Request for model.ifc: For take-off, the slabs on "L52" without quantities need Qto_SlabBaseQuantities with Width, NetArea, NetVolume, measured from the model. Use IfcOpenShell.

First a look at what the model holds.

```python
import ifcopenshell
import ifcopenshell.util.element
import ifcopenshell.util.unit

model = ifcopenshell.open("model.ifc")
print(model.schema)
for unit_type in ("LENGTHUNIT", "AREAUNIT", "VOLUMEUNIT"):
    print(unit_type, ifcopenshell.util.unit.calculate_unit_scale(model, unit_type))
storey = next(s for s in model.by_type("IfcBuildingStorey") if s.Name == "L52")
slabs = [e for e in ifcopenshell.util.element.get_decomposition(storey) if e.is_a("IfcSlab")]
for e in sorted(slabs, key=lambda e: e.id()):
    print(e.id(), e.is_a(), e.Name, list(ifcopenshell.util.element.get_psets(e, qtos_only=True)), sep=" | ")
```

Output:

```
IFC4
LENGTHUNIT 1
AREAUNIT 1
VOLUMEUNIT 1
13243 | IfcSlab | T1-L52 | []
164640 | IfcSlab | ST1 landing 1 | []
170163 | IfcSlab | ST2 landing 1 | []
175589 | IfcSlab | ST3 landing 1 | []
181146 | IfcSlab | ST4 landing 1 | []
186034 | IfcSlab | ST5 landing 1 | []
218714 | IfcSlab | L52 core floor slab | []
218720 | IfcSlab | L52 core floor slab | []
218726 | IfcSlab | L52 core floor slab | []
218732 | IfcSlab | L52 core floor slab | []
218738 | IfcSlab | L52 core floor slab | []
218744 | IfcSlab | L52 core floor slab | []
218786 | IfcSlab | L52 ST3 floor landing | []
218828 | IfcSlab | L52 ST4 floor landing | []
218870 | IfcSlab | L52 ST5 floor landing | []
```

```python
import ifcopenshell
import ifcopenshell.api.pset
import ifcopenshell.geom
import ifcopenshell.util.element
import ifcopenshell.util.shape
import ifcopenshell.util.unit

model = ifcopenshell.open("model.ifc")
unit_scale = ifcopenshell.util.unit.calculate_unit_scale(model)
area_scale = ifcopenshell.util.unit.calculate_unit_scale(model, "AREAUNIT")
volume_scale = ifcopenshell.util.unit.calculate_unit_scale(model, "VOLUMEUNIT")
settings = ifcopenshell.geom.settings()

storey = next(s for s in model.by_type("IfcBuildingStorey") if s.Name == "L52")
slabs = [e for e in ifcopenshell.util.element.get_decomposition(storey) if e.is_a("IfcSlab")]

for e in sorted(slabs, key=lambda e: e.id()):
    if ifcopenshell.util.element.get_psets(e, qtos_only=True, should_inherit=False):
        continue
    # Geometry comes back in metres, in the element's own axes.
    shape = ifcopenshell.geom.create_shape(settings, e)
    values = {
        "Width": ifcopenshell.util.shape.get_z(shape.geometry) / unit_scale,
        "NetArea": ifcopenshell.util.shape.get_footprint_area(shape.geometry) / area_scale,
        "NetVolume": ifcopenshell.util.shape.get_volume(shape.geometry) / volume_scale,
    }
    qto = ifcopenshell.api.pset.add_qto(model, product=e, name="Qto_SlabBaseQuantities")
    ifcopenshell.api.pset.edit_qto(model, qto=qto, properties=values)
    print(e.id(), {k: round(v, 3) for k, v in values.items()})

model.write("model-out.ifc")
```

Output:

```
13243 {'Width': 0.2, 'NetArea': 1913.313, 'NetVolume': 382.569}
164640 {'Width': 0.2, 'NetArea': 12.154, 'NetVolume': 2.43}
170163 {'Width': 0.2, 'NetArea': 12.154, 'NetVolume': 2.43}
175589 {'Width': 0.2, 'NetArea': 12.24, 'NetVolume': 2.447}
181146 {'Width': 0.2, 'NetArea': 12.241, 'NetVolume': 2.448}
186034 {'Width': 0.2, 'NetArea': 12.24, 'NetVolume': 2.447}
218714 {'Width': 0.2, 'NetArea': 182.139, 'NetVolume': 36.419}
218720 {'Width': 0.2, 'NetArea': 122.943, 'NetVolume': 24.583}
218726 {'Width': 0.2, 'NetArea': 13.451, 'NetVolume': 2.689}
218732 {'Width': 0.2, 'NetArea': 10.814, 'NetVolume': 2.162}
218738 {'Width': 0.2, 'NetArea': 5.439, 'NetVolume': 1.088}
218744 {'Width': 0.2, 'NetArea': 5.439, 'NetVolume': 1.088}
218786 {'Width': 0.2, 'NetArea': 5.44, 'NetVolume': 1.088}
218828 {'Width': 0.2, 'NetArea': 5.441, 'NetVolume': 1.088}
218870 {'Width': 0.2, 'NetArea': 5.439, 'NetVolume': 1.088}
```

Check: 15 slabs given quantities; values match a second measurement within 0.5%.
